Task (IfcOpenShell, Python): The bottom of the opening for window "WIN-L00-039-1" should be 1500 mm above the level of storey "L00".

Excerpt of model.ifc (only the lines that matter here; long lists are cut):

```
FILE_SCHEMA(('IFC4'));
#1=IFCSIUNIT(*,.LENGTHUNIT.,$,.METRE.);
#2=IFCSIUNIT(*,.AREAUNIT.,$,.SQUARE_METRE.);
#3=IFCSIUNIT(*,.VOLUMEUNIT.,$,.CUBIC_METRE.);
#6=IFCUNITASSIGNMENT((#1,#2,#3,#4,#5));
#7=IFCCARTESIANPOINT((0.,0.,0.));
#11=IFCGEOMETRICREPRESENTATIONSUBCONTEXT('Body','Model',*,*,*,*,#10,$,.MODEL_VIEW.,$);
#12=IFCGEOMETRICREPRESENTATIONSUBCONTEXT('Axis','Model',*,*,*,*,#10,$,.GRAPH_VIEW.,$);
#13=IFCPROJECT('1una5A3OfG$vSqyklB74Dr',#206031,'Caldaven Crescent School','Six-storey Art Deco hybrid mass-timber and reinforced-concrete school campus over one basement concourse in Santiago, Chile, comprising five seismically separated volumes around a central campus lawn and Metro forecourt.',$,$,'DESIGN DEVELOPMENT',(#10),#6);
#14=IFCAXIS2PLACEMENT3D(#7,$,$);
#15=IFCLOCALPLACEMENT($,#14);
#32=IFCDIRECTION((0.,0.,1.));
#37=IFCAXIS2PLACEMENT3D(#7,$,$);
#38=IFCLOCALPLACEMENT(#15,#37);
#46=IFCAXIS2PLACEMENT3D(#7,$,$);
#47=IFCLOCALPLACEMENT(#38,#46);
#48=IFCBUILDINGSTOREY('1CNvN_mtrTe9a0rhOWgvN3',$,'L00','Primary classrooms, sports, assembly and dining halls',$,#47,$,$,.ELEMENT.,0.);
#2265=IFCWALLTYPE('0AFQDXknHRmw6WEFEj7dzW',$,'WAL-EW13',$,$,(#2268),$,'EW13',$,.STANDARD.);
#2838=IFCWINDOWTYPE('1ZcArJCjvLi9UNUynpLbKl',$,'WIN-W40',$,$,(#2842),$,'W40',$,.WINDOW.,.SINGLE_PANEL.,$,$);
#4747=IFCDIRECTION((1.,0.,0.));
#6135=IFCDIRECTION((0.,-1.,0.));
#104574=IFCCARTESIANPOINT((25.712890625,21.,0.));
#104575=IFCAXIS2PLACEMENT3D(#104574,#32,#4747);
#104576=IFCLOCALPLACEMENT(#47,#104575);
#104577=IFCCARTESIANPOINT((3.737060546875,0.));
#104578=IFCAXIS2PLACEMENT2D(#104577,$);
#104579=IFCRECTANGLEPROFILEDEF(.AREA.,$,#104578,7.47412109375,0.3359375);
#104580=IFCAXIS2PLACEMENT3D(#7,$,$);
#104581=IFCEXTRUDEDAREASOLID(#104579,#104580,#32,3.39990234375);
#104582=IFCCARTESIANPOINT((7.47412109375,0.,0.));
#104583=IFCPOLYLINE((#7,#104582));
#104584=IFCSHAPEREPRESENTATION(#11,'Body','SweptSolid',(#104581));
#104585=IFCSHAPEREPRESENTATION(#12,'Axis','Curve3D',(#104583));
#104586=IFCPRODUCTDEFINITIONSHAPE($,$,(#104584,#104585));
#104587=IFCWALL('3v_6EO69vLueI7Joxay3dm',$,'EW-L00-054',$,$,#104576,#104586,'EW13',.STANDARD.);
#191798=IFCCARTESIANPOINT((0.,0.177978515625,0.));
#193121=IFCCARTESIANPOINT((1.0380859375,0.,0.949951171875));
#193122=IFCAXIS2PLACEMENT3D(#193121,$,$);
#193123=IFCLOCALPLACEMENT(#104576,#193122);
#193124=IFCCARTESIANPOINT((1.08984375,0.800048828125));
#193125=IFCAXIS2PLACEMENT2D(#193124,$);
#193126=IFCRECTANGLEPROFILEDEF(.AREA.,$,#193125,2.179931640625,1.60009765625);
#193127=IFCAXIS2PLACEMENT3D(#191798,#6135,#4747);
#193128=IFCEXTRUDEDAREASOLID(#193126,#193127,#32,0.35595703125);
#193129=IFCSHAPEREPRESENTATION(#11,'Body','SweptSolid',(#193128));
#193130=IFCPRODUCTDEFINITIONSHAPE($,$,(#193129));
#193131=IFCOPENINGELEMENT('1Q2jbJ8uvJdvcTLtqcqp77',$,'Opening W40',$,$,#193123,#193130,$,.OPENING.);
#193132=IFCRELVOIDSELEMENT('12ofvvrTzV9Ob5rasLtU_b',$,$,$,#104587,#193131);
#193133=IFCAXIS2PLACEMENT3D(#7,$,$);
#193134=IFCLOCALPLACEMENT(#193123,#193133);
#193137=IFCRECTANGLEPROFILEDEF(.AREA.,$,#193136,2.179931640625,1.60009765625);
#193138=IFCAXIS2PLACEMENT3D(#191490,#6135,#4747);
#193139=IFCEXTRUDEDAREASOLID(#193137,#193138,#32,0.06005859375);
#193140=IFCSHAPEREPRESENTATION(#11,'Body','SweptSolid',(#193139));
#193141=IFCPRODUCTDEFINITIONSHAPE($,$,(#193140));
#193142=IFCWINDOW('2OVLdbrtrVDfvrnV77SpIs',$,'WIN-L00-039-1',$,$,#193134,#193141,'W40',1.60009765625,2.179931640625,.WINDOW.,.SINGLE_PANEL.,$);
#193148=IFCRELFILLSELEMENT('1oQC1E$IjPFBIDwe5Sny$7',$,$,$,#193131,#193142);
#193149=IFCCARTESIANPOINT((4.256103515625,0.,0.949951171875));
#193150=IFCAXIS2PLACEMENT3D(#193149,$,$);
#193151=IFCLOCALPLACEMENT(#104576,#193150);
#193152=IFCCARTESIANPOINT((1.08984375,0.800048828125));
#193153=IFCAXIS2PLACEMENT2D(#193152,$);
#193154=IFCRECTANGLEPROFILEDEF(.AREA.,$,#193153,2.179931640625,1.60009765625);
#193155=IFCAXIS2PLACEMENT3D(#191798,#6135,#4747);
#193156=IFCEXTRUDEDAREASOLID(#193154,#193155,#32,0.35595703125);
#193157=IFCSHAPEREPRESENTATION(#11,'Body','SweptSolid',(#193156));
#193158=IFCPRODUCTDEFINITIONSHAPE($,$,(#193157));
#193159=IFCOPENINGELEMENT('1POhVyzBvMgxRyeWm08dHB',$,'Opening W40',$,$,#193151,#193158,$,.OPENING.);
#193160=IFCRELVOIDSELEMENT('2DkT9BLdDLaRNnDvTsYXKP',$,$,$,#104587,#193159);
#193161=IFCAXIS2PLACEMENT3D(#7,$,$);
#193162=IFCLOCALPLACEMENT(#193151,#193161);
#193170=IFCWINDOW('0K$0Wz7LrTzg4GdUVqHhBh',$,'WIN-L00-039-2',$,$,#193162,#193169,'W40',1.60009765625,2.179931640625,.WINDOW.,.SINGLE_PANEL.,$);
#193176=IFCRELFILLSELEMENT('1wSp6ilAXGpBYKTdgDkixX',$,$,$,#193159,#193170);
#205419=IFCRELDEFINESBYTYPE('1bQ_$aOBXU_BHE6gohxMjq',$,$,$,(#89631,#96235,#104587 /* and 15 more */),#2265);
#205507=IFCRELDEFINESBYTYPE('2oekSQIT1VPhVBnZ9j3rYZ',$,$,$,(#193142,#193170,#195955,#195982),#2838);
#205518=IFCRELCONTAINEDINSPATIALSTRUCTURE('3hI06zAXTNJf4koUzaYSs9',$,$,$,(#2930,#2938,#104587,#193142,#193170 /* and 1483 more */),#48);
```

```python
import numpy as np
import ifcopenshell
import ifcopenshell.api.geometry
import ifcopenshell.geom
import ifcopenshell.util.element
import ifcopenshell.util.placement
import ifcopenshell.util.shape
import ifcopenshell.util.unit

model = ifcopenshell.open("model.ifc")
unit_scale = ifcopenshell.util.unit.calculate_unit_scale(model)

window = model.by_guid("2OVLdbrtrVDfvrnV77SpIs")
opening = window.FillsVoids[0].RelatingOpeningElement
storey = ifcopenshell.util.element.get_container(window, ifc_class="IfcBuildingStorey")
level = ifcopenshell.util.placement.get_local_placement(storey.ObjectPlacement)[2, 3]

# The opening's origin need not be at the sill, so measure its lowest point.
shape = ifcopenshell.geom.create_shape(ifcopenshell.geom.settings(), opening)
bottom = ifcopenshell.util.shape.get_shape_bottom_elevation(shape, shape.geometry) / unit_scale
dz = level + 1.5 - bottom

shift = np.array([0.0, 0.0, dz])
# The window is placed relative to its opening, so it follows when the opening moves.
matrix = ifcopenshell.util.placement.get_local_placement(opening.ObjectPlacement)
matrix[:3, 3] += shift
ifcopenshell.api.geometry.edit_object_placement(
    model, product=opening, matrix=matrix, is_si=False, should_transform_children=True
)

print(f"moved by {dz * unit_scale:+.3f} m")

model.write("model_edited.ifc")
```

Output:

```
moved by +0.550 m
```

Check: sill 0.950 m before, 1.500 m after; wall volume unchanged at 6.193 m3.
